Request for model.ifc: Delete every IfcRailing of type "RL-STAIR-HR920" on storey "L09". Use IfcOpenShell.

First a look at what the model holds.

```python
import ifcopenshell
import ifcopenshell.util.element

model = ifcopenshell.open("model.ifc")
print(model.schema)
storey = next(s for s in model.by_type("IfcBuildingStorey") if s.Name == "L09")
railings = [e for e in ifcopenshell.util.element.get_decomposition(storey) if e.is_a("IfcRailing")]
seen = {}
for e in railings:
    element_type = ifcopenshell.util.element.get_type(e)
    name = element_type.Name if element_type not in (None, e) else None
    seen[name] = seen.get(name, 0) + 1
for name, count in sorted(seen.items(), key=str):
    print(count, "x", name)
```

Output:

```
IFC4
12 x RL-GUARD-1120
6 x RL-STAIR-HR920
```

```python
import ifcopenshell
import ifcopenshell.api.root
import ifcopenshell.util.element

model = ifcopenshell.open("model.ifc")

storey = next(s for s in model.by_type("IfcBuildingStorey") if s.Name == "L09")
railings = [e for e in ifcopenshell.util.element.get_decomposition(storey) if e.is_a("IfcRailing")]
targets = [e for e in railings if (t := ifcopenshell.util.element.get_type(e)) not in (None, e) and t.Name == "RL-STAIR-HR920"]

for e in targets:
    ifcopenshell.api.root.remove_product(model, product=e)
print(len(targets), "removed")

model.write("model-out.ifc")
```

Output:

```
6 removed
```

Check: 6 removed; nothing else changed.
